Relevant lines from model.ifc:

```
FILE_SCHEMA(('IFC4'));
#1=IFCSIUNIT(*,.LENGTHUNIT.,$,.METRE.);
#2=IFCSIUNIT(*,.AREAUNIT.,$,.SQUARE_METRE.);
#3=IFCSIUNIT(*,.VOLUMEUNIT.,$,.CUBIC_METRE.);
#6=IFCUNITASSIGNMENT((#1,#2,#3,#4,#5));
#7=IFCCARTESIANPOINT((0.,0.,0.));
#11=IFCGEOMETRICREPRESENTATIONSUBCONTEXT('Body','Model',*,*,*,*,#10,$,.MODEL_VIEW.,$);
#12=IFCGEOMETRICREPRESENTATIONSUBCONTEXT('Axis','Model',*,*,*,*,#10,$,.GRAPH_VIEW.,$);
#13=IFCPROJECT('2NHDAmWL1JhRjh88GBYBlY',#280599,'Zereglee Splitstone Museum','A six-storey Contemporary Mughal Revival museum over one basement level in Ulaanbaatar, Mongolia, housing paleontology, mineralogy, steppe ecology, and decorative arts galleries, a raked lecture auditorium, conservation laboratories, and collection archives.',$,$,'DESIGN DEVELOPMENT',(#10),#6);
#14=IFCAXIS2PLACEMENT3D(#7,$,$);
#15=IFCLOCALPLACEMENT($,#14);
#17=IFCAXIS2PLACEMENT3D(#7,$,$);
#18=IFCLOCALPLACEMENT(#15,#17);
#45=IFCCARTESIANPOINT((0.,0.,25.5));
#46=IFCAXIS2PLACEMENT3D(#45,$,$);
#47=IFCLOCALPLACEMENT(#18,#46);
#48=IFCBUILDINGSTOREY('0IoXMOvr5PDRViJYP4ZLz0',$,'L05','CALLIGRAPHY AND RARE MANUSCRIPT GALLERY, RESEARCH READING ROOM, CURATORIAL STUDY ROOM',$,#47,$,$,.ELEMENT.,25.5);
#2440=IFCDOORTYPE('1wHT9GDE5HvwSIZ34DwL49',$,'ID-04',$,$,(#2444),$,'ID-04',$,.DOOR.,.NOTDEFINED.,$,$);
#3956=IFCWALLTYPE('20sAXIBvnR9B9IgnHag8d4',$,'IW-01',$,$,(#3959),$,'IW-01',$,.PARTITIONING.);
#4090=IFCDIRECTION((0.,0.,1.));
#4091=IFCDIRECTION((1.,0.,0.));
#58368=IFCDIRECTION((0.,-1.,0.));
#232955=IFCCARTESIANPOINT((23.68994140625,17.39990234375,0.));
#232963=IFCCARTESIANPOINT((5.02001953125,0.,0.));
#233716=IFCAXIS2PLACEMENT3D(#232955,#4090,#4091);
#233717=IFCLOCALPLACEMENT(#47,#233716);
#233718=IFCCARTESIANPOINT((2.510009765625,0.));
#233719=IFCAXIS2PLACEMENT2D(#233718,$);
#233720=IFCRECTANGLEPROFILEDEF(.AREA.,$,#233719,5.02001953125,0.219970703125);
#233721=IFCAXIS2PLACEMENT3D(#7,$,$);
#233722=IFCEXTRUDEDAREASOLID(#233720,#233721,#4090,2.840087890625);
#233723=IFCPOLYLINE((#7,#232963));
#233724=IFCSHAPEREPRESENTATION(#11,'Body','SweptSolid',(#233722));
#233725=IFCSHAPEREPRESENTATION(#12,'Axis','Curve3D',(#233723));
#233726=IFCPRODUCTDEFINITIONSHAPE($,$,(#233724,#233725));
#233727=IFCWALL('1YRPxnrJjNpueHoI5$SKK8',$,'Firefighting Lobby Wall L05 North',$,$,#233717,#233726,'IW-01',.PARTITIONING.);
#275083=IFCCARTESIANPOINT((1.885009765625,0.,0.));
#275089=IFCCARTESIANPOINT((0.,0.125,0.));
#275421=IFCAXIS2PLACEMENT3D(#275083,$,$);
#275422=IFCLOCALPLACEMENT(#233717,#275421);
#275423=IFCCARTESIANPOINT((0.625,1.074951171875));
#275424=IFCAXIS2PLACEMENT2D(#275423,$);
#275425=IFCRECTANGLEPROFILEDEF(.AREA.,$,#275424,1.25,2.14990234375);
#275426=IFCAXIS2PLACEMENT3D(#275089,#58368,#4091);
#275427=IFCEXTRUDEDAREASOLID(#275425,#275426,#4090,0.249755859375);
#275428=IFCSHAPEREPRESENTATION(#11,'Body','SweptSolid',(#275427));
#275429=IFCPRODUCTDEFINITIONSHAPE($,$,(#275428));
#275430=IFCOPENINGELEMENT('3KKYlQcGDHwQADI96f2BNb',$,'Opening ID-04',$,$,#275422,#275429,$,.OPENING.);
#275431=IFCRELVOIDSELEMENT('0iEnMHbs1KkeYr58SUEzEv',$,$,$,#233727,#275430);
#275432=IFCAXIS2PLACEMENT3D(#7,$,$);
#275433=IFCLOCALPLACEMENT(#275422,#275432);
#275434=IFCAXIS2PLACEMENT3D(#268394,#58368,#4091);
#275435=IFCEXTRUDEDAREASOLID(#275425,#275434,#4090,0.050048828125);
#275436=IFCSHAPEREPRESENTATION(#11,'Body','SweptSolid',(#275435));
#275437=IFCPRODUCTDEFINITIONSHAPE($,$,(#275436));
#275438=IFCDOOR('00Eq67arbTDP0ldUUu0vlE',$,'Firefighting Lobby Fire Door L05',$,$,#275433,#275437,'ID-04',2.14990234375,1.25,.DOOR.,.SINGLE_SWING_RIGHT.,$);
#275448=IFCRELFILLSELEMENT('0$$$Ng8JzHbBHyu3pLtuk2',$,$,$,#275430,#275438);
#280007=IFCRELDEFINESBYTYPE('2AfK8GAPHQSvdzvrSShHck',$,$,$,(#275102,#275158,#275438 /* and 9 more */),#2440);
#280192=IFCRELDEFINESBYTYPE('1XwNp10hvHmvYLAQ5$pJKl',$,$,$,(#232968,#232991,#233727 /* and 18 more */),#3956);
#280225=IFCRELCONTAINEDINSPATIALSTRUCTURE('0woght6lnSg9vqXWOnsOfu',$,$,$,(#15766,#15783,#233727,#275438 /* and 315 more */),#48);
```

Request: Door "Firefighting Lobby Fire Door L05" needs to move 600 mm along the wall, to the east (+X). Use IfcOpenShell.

```python
import ifcopenshell
import ifcopenshell.api.geometry
import ifcopenshell.util.placement
import ifcopenshell.util.unit

model = ifcopenshell.open("model.ifc")
unit_scale = ifcopenshell.util.unit.calculate_unit_scale(model)

door = model.by_guid("00Eq67arbTDP0ldUUu0vlE")
opening = door.FillsVoids[0].RelatingOpeningElement
wall = opening.VoidsElements[0].RelatingBuildingElement

wall_matrix = ifcopenshell.util.placement.get_local_placement(wall.ObjectPlacement)
shift = wall_matrix[:3, 0] * 0.6 / unit_scale
before = ifcopenshell.util.placement.get_local_placement(door.ObjectPlacement)[:3, 3].copy()

# The door is placed relative to its opening, so it follows when the opening moves.
matrix = ifcopenshell.util.placement.get_local_placement(opening.ObjectPlacement)
matrix[:3, 3] += shift
ifcopenshell.api.geometry.edit_object_placement(
    model, product=opening, matrix=matrix, is_si=False, should_transform_children=True
)

after = ifcopenshell.util.placement.get_local_placement(door.ObjectPlacement)[:3, 3]
print("door moved by", (after - before).round(3) + 0.0)

model.write("model_updated.ifc")
```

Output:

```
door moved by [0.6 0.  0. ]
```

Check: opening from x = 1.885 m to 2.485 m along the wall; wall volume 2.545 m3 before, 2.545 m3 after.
